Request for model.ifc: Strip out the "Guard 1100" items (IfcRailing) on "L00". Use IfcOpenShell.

First a look at what the model holds.

```python
import ifcopenshell
import ifcopenshell.util.element

model = ifcopenshell.open("model.ifc")
print(model.schema)
storey = next(s for s in model.by_type("IfcBuildingStorey") if s.Name == "L00")
railings = [e for e in ifcopenshell.util.element.get_decomposition(storey) if e.is_a("IfcRailing")]
seen = {}
for e in railings:
    element_type = ifcopenshell.util.element.get_type(e)
    name = element_type.Name if element_type not in (None, e) else None
    seen[name] = seen.get(name, 0) + 1
for name, count in sorted(seen.items(), key=str):
    print(count, "x", name)
```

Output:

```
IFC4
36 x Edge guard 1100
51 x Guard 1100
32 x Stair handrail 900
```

```python
import ifcopenshell
import ifcopenshell.api.root
import ifcopenshell.util.element

model = ifcopenshell.open("model.ifc")

storey = next(s for s in model.by_type("IfcBuildingStorey") if s.Name == "L00")
railings = [e for e in ifcopenshell.util.element.get_decomposition(storey) if e.is_a("IfcRailing")]
targets = [e for e in railings if (t := ifcopenshell.util.element.get_type(e)) not in (None, e) and t.Name == "Guard 1100"]

for e in targets:
    ifcopenshell.api.root.remove_product(model, product=e)
print(len(targets), "removed")

model.write("model_v2.ifc")
```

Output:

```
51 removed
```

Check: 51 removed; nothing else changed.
